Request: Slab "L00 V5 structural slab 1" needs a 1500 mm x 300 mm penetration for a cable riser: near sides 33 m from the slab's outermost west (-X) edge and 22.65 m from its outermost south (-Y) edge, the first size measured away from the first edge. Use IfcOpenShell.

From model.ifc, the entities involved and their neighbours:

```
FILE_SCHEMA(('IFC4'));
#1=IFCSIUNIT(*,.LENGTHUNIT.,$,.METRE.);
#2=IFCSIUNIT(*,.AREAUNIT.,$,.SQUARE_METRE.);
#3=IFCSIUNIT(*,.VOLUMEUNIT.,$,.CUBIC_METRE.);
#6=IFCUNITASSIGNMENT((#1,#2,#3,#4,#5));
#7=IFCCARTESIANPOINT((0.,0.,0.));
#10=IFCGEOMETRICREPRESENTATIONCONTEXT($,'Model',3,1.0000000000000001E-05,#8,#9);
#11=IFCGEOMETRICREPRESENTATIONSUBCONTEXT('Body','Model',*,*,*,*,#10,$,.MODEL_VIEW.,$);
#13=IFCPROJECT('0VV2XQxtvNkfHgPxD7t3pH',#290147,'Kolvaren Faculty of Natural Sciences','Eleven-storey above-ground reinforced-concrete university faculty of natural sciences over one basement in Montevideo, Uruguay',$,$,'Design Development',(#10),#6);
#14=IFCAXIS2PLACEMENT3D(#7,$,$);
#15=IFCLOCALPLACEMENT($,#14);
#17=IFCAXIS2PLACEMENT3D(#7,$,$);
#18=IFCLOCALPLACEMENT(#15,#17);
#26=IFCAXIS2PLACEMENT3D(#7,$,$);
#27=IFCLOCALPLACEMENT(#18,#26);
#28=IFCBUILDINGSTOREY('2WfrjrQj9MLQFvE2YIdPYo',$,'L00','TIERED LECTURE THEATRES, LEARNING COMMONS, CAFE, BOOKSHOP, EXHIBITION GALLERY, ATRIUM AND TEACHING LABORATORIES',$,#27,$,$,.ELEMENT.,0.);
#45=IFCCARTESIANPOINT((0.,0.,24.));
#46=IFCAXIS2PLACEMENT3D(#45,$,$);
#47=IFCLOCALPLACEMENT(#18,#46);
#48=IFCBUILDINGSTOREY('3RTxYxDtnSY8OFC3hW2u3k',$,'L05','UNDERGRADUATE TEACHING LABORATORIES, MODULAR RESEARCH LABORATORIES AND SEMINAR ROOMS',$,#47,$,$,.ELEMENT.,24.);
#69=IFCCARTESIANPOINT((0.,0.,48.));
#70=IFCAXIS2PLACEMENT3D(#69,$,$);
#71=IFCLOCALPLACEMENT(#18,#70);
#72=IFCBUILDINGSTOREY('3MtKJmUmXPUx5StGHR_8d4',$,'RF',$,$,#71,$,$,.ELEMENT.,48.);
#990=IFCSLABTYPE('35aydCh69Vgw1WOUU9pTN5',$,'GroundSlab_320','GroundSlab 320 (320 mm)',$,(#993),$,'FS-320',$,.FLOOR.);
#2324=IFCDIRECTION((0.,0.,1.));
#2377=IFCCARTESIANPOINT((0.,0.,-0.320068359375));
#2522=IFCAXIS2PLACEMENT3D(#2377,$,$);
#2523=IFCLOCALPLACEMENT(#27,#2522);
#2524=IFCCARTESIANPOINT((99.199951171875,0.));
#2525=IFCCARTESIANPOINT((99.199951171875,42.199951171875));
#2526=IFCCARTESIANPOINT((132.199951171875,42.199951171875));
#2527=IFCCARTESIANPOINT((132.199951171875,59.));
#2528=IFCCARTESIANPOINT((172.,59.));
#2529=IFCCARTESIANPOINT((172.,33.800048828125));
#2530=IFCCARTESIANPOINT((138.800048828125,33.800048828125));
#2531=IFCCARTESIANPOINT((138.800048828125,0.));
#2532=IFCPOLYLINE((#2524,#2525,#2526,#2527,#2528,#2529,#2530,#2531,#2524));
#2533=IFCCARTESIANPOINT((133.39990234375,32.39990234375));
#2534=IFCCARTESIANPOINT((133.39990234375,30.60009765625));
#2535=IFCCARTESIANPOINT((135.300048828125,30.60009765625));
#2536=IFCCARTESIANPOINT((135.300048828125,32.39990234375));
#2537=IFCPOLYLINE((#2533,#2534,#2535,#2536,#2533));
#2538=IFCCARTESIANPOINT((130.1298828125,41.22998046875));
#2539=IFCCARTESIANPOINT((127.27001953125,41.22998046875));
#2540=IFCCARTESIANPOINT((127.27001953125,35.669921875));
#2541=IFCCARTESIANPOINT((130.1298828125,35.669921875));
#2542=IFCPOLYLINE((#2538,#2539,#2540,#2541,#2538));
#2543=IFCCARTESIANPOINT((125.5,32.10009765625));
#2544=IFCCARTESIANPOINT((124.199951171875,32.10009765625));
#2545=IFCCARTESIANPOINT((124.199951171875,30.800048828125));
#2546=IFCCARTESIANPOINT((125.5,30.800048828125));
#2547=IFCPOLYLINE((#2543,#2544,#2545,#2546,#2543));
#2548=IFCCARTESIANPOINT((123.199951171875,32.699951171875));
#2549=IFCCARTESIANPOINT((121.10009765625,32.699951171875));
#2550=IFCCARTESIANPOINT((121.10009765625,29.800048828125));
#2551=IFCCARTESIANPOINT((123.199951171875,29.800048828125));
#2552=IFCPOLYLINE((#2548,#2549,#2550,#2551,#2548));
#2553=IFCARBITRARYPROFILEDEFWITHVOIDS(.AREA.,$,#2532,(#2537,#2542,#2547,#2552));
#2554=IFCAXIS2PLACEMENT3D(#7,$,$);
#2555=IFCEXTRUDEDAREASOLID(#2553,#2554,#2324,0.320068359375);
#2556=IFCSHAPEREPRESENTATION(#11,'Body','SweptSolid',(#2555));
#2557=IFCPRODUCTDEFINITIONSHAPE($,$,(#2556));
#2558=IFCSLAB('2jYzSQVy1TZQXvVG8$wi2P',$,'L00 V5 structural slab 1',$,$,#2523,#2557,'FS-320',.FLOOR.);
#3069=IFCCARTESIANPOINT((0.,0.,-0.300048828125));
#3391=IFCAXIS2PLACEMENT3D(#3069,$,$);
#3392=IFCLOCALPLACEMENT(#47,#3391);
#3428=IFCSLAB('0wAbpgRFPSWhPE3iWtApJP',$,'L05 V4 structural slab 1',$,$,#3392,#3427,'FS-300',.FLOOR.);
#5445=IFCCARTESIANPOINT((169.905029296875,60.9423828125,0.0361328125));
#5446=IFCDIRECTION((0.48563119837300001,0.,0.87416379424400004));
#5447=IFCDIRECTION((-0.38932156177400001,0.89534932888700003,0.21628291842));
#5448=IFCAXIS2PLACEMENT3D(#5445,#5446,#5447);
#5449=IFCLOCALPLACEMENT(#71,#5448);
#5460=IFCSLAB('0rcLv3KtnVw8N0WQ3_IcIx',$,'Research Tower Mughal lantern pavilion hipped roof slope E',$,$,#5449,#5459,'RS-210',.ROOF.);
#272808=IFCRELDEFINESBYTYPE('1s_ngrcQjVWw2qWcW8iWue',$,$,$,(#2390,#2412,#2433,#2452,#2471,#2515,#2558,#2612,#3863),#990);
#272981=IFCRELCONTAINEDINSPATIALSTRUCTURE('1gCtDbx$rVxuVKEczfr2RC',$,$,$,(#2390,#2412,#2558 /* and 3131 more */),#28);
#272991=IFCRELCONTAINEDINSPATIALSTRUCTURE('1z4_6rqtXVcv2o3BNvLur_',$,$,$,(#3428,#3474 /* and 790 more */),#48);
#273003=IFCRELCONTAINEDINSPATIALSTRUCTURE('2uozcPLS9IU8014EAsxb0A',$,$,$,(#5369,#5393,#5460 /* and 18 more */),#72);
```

```python
import numpy as np
import ifcopenshell
import ifcopenshell.api.feature
import ifcopenshell.api.geometry
import ifcopenshell.api.root
import ifcopenshell.geom
import ifcopenshell.util.placement
import ifcopenshell.util.representation
import ifcopenshell.util.shape
import ifcopenshell.util.unit

model = ifcopenshell.open("model.ifc")
unit_scale = ifcopenshell.util.unit.calculate_unit_scale(model)
settings = ifcopenshell.geom.settings()


def volume(element):
    """Net volume in cubic metres, openings subtracted."""
    shape = ifcopenshell.geom.create_shape(settings, element)
    return ifcopenshell.util.shape.get_volume(shape.geometry)


slab = model.by_id(2558)
before = volume(slab)

# Extent in the slab's own axes, in metres. The edges named are its -X and -Y sides.
slab_shape = ifcopenshell.geom.create_shape(settings, slab)
vertices = ifcopenshell.util.shape.get_vertices(slab_shape.geometry)
x_min, y_min, bottom = vertices.min(axis=0)
top = vertices[:, 2].max()

opening = ifcopenshell.api.root.create_entity(model, ifc_class="IfcOpeningElement", name="Cable riser opening", predefined_type="OPENING")
context = ifcopenshell.util.representation.get_context(model, "Model", "Body", "MODEL_VIEW")
width, depth = 1.5, 0.3
outline = [(0.0, 0.0), (width, 0.0), (width, depth), (0.0, depth), (0.0, 0.0)]
# Overshoot both faces by 50 mm so the cut is clean.
shape = ifcopenshell.api.geometry.add_slab_representation(
    model, context=context, depth=top - bottom + 0.1, polyline=outline
)
ifcopenshell.api.geometry.assign_representation(model, product=opening, representation=shape)

matrix = ifcopenshell.util.placement.get_local_placement(slab.ObjectPlacement)
matrix[:, 3] = matrix @ np.append(np.array([x_min + 33, y_min + 22.65, bottom - 0.05]) / unit_scale, 1.0)
ifcopenshell.api.geometry.edit_object_placement(model, product=opening, matrix=matrix, is_si=False)
ifcopenshell.api.feature.add_feature(model, feature=opening, element=slab)

after = volume(slab)

print(f"slab volume {before:.3f} -> {after:.3f} m3")

model.write("model_v2.ifc")
```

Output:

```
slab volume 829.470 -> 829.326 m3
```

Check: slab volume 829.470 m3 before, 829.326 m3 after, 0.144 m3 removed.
